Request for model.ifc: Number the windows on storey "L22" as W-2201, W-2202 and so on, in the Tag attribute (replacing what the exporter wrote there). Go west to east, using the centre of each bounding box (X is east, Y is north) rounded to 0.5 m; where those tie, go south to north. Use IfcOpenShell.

First a look at what the model holds.

```python
import ifcopenshell
import ifcopenshell.util.element
import ifcopenshell.util.placement

model = ifcopenshell.open("model.ifc")
print(model.schema)
storey = next(s for s in model.by_type("IfcBuildingStorey") if s.Name == "L22")
windows = [e for e in ifcopenshell.util.element.get_decomposition(storey) if e.is_a("IfcWindow")]
for e in sorted(windows, key=lambda e: e.id()):
    origin = ifcopenshell.util.placement.get_local_placement(e.ObjectPlacement)[:3, 3]
    print(e.id(), e.Tag, e.Name, origin.round(2) + 0.0, sep=" | ")
```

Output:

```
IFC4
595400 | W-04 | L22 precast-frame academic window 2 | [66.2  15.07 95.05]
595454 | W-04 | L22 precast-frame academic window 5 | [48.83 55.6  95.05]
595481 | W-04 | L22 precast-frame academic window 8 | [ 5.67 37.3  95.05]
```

```python
import ifcopenshell
import ifcopenshell.geom
import ifcopenshell.util.element
import ifcopenshell.util.shape

model = ifcopenshell.open("model.ifc")
settings = ifcopenshell.geom.settings()
settings.set("use-world-coords", True)


def centre(element):
    shape = ifcopenshell.geom.create_shape(settings, element)
    return ifcopenshell.util.shape.get_bbox_centroid(shape.geometry)


storey = next(s for s in model.by_type("IfcBuildingStorey") if s.Name == "L22")
windows = [e for e in ifcopenshell.util.element.get_decomposition(storey) if e.is_a("IfcWindow")]

# Insertion points can sit at a corner or the storey origin, so sort by the geometry (in metres).
centres = {e: centre(e) for e in windows}
windows.sort(key=lambda e: (round(centres[e][0] / 0.5), centres[e][1]))

for i, e in enumerate(windows, start=1):
    number = f"W-22{i:02d}"
    e.Tag = number
    print(e.id(), number)

model.write("model_rev.ifc")
```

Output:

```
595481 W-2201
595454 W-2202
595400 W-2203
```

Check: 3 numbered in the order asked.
